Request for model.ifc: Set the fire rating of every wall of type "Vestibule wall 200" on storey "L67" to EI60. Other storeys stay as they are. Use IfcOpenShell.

First a look at what the model holds.

```python
import ifcopenshell
import ifcopenshell.util.element

model = ifcopenshell.open("model.ifc")
print(model.schema)
storey = next(s for s in model.by_type("IfcBuildingStorey") if s.Name == "L67")
walls = [e for e in ifcopenshell.util.element.get_decomposition(storey) if e.is_a("IfcWall")]
seen = {}
for e in walls:
    element_type = ifcopenshell.util.element.get_type(e)
    key = (element_type.Name if element_type != e and element_type else None, ifcopenshell.util.element.get_pset(e, "Pset_WallCommon", "FireRating"))
    seen[key] = seen.get(key, 0) + 1
for (name, value), count in sorted(seen.items(), key=str):
    print(count, "x", name, "|", value)
```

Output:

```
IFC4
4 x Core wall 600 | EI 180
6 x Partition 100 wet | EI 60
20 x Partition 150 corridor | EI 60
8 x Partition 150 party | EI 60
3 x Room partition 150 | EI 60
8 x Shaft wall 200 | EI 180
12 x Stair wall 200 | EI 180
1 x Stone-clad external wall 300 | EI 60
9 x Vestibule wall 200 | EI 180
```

```python
import ifcopenshell
import ifcopenshell.api.pset
import ifcopenshell.util.element

model = ifcopenshell.open("model.ifc")

storey = next(s for s in model.by_type("IfcBuildingStorey") if s.Name == "L67")
walls = [e for e in ifcopenshell.util.element.get_decomposition(storey) if e.is_a("IfcWall")]

count = 0
for e in walls:
    element_type = ifcopenshell.util.element.get_type(e)
    if element_type in (None, e) or element_type.Name != "Vestibule wall 200":
        continue
    found = ifcopenshell.util.element.get_pset(e, "Pset_WallCommon", should_inherit=False)
    if found:
        pset = model.by_id(found["id"])
        if len(ifcopenshell.util.element.get_elements_by_pset(pset)) > 1:
            pset = ifcopenshell.api.pset.unshare_pset(model, products=[e], pset=pset)[0]
    else:
        pset = ifcopenshell.api.pset.add_pset(model, product=e, name="Pset_WallCommon")
    ifcopenshell.api.pset.edit_pset(model, pset=pset, properties={"FireRating": "EI60"})
    count += 1

print(count, "walls updated")

model.write("model-out.ifc")
```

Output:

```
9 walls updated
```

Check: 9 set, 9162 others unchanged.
